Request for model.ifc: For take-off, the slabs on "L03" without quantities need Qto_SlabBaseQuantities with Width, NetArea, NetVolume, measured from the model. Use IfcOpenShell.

First a look at what the model holds.

```python
import ifcopenshell
import ifcopenshell.util.element
import ifcopenshell.util.unit

model = ifcopenshell.open("model.ifc")
print(model.schema)
for unit_type in ("LENGTHUNIT", "AREAUNIT", "VOLUMEUNIT"):
    print(unit_type, ifcopenshell.util.unit.calculate_unit_scale(model, unit_type))
storey = next(s for s in model.by_type("IfcBuildingStorey") if s.Name == "L03")
slabs = [e for e in ifcopenshell.util.element.get_decomposition(storey) if e.is_a("IfcSlab")]
for e in sorted(slabs, key=lambda e: e.id()):
    print(e.id(), e.is_a(), e.Name, list(ifcopenshell.util.element.get_psets(e, qtos_only=True)), sep=" | ")
```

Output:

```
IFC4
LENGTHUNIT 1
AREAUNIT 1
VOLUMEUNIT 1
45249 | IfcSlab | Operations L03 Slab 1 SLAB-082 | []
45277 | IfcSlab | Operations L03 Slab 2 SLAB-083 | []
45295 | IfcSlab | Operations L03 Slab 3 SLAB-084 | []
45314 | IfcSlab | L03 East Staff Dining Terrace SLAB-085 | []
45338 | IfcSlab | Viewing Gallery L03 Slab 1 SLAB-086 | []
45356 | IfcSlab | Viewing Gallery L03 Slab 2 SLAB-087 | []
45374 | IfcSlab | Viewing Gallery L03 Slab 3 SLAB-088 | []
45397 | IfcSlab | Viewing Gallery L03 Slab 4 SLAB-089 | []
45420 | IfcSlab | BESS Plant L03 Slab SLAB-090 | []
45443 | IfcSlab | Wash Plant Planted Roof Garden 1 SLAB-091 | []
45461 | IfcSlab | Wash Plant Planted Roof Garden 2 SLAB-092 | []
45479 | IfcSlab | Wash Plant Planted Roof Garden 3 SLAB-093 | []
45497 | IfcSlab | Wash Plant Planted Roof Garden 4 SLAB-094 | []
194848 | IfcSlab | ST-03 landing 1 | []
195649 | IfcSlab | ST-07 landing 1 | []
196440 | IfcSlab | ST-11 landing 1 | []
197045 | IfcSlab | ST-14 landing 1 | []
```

```python
import ifcopenshell
import ifcopenshell.api.pset
import ifcopenshell.geom
import ifcopenshell.util.element
import ifcopenshell.util.shape
import ifcopenshell.util.unit

model = ifcopenshell.open("model.ifc")
unit_scale = ifcopenshell.util.unit.calculate_unit_scale(model)
area_scale = ifcopenshell.util.unit.calculate_unit_scale(model, "AREAUNIT")
volume_scale = ifcopenshell.util.unit.calculate_unit_scale(model, "VOLUMEUNIT")
settings = ifcopenshell.geom.settings()

storey = next(s for s in model.by_type("IfcBuildingStorey") if s.Name == "L03")
slabs = [e for e in ifcopenshell.util.element.get_decomposition(storey) if e.is_a("IfcSlab")]

for e in sorted(slabs, key=lambda e: e.id()):
    if ifcopenshell.util.element.get_psets(e, qtos_only=True, should_inherit=False):
        continue
    # Geometry comes back in metres, in the element's own axes.
    shape = ifcopenshell.geom.create_shape(settings, e)
    values = {
        "Width": ifcopenshell.util.shape.get_z(shape.geometry) / unit_scale,
        "NetArea": ifcopenshell.util.shape.get_footprint_area(shape.geometry) / area_scale,
        "NetVolume": ifcopenshell.util.shape.get_volume(shape.geometry) / volume_scale,
    }
    qto = ifcopenshell.api.pset.add_qto(model, product=e, name="Qto_SlabBaseQuantities")
    ifcopenshell.api.pset.edit_qto(model, qto=qto, properties=values)
    print(e.id(), {k: round(v, 3) for k, v in values.items()})

model.write("model_updated.ifc")
```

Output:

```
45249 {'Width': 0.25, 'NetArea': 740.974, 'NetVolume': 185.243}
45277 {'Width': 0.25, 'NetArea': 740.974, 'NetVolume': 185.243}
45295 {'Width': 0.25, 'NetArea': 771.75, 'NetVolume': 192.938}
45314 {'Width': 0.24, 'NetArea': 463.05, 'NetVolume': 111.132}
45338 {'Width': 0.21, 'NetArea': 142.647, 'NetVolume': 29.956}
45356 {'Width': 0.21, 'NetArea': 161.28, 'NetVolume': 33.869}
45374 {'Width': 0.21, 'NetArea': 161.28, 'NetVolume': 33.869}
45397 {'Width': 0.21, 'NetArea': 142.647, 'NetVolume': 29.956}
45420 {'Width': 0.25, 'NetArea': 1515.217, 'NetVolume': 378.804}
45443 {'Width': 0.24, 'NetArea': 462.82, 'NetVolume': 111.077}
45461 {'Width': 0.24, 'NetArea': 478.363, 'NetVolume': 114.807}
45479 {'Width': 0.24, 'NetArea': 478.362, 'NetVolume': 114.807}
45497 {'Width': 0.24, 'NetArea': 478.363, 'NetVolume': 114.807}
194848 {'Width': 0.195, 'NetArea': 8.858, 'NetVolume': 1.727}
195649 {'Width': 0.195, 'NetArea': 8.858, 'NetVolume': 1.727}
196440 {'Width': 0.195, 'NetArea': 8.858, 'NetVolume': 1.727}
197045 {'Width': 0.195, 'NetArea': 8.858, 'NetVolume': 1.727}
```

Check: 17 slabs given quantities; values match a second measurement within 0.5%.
